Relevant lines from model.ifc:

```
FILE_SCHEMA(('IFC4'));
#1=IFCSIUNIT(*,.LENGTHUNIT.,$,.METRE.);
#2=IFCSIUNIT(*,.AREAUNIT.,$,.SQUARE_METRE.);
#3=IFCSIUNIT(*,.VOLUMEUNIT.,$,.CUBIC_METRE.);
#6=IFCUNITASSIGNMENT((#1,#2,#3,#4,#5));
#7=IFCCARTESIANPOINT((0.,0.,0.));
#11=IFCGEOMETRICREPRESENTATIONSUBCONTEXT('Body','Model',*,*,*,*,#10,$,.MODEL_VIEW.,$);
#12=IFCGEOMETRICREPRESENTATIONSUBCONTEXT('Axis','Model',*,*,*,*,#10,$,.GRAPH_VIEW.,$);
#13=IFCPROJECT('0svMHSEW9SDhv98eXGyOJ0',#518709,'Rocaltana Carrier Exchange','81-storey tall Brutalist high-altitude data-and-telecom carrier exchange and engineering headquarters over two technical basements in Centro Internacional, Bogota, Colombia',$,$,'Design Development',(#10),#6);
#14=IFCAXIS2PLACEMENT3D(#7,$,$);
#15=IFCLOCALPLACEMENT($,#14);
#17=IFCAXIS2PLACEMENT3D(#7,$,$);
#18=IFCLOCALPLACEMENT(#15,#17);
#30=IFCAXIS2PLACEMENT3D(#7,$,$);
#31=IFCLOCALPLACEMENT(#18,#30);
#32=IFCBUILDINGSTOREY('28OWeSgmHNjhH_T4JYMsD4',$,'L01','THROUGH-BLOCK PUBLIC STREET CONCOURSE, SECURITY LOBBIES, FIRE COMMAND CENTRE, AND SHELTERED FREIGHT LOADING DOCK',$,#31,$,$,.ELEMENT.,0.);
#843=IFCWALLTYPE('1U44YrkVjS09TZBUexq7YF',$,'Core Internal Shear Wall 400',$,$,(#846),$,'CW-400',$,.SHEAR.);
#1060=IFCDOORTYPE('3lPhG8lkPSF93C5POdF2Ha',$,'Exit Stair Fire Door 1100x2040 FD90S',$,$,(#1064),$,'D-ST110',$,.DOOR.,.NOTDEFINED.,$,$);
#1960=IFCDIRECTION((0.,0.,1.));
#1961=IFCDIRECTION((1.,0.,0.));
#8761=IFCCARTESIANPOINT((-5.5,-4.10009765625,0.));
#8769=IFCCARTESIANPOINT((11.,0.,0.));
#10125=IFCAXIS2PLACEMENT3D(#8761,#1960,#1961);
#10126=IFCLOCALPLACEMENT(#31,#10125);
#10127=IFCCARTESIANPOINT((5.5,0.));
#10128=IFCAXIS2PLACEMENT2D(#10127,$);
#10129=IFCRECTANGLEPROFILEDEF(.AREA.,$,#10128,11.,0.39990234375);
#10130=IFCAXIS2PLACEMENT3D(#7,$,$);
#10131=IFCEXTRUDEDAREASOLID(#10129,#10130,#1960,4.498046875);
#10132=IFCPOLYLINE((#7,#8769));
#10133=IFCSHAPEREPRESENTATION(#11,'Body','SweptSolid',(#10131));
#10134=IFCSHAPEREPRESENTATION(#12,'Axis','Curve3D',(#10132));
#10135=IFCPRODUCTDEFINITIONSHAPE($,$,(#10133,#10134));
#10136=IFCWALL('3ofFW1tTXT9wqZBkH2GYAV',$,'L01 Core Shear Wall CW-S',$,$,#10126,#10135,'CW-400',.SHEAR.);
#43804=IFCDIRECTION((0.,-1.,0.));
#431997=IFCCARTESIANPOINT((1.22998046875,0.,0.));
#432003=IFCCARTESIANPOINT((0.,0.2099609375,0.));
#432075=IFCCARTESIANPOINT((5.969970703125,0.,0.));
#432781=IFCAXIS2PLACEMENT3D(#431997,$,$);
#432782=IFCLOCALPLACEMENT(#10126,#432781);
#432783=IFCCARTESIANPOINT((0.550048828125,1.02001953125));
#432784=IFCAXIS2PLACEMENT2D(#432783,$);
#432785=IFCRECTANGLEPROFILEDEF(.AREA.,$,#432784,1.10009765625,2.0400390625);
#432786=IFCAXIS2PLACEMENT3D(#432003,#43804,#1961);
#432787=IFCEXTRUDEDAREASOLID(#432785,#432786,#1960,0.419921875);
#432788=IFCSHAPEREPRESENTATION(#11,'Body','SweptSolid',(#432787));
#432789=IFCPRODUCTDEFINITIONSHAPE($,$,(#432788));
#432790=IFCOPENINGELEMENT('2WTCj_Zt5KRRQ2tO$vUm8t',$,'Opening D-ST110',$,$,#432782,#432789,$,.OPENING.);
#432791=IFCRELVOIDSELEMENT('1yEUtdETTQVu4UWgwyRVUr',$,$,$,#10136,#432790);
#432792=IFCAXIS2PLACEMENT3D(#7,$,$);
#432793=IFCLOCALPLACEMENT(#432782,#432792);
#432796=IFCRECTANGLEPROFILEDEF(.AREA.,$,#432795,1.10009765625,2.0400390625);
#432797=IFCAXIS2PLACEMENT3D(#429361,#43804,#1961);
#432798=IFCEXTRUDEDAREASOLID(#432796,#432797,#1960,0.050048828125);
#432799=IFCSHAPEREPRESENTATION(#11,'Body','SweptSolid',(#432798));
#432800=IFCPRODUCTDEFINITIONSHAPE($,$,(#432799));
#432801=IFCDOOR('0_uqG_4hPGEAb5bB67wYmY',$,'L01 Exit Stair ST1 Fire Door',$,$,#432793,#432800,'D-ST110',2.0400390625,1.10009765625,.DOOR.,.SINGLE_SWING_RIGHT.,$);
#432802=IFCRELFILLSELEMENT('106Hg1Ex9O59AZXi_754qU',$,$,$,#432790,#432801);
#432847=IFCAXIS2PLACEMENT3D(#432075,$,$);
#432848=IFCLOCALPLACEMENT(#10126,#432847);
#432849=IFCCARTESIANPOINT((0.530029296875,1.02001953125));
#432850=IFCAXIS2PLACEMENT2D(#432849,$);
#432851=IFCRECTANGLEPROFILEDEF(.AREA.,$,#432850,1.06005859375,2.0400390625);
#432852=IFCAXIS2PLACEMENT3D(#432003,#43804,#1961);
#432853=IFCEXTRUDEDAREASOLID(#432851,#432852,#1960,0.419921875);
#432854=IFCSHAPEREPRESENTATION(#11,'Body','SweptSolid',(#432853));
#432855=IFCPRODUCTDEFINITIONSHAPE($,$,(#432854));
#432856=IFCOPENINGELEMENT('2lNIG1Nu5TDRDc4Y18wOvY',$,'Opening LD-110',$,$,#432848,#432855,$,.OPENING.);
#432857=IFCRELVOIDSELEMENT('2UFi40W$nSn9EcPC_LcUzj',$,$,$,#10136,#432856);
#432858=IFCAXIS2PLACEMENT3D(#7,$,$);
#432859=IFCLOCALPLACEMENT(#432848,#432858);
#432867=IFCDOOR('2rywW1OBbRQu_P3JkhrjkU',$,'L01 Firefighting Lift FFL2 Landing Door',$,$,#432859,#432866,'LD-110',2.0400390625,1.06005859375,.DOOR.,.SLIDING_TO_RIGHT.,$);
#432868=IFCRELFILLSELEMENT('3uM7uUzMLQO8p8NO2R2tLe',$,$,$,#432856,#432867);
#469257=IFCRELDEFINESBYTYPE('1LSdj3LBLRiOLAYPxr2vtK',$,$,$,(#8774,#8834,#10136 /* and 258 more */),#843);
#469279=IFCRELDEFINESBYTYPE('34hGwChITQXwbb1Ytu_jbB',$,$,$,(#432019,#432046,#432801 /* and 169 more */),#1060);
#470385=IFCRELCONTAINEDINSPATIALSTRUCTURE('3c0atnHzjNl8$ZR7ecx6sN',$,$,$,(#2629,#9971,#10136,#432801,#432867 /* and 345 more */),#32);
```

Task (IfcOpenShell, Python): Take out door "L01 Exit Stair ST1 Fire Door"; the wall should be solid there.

```python
import ifcopenshell
import ifcopenshell.api.feature
import ifcopenshell.api.root
import ifcopenshell.geom
import ifcopenshell.util.shape

model = ifcopenshell.open("model.ifc")
settings = ifcopenshell.geom.settings()


def volume(element):
    """Net volume in cubic metres, openings subtracted."""
    shape = ifcopenshell.geom.create_shape(settings, element)
    return ifcopenshell.util.shape.get_volume(shape.geometry)


door = model.by_guid("0_uqG_4hPGEAb5bB67wYmY")
opening = door.FillsVoids[0].RelatingOpeningElement
wall = opening.VoidsElements[0].RelatingBuildingElement
before = volume(wall)

ifcopenshell.api.root.remove_product(model, product=door)
ifcopenshell.api.feature.remove_feature(model, feature=opening)

after = volume(wall)

print(f"wall volume {before:.3f} -> {after:.3f} m3")

model.write("model_edited.ifc")
```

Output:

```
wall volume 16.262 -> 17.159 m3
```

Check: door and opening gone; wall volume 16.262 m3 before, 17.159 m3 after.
